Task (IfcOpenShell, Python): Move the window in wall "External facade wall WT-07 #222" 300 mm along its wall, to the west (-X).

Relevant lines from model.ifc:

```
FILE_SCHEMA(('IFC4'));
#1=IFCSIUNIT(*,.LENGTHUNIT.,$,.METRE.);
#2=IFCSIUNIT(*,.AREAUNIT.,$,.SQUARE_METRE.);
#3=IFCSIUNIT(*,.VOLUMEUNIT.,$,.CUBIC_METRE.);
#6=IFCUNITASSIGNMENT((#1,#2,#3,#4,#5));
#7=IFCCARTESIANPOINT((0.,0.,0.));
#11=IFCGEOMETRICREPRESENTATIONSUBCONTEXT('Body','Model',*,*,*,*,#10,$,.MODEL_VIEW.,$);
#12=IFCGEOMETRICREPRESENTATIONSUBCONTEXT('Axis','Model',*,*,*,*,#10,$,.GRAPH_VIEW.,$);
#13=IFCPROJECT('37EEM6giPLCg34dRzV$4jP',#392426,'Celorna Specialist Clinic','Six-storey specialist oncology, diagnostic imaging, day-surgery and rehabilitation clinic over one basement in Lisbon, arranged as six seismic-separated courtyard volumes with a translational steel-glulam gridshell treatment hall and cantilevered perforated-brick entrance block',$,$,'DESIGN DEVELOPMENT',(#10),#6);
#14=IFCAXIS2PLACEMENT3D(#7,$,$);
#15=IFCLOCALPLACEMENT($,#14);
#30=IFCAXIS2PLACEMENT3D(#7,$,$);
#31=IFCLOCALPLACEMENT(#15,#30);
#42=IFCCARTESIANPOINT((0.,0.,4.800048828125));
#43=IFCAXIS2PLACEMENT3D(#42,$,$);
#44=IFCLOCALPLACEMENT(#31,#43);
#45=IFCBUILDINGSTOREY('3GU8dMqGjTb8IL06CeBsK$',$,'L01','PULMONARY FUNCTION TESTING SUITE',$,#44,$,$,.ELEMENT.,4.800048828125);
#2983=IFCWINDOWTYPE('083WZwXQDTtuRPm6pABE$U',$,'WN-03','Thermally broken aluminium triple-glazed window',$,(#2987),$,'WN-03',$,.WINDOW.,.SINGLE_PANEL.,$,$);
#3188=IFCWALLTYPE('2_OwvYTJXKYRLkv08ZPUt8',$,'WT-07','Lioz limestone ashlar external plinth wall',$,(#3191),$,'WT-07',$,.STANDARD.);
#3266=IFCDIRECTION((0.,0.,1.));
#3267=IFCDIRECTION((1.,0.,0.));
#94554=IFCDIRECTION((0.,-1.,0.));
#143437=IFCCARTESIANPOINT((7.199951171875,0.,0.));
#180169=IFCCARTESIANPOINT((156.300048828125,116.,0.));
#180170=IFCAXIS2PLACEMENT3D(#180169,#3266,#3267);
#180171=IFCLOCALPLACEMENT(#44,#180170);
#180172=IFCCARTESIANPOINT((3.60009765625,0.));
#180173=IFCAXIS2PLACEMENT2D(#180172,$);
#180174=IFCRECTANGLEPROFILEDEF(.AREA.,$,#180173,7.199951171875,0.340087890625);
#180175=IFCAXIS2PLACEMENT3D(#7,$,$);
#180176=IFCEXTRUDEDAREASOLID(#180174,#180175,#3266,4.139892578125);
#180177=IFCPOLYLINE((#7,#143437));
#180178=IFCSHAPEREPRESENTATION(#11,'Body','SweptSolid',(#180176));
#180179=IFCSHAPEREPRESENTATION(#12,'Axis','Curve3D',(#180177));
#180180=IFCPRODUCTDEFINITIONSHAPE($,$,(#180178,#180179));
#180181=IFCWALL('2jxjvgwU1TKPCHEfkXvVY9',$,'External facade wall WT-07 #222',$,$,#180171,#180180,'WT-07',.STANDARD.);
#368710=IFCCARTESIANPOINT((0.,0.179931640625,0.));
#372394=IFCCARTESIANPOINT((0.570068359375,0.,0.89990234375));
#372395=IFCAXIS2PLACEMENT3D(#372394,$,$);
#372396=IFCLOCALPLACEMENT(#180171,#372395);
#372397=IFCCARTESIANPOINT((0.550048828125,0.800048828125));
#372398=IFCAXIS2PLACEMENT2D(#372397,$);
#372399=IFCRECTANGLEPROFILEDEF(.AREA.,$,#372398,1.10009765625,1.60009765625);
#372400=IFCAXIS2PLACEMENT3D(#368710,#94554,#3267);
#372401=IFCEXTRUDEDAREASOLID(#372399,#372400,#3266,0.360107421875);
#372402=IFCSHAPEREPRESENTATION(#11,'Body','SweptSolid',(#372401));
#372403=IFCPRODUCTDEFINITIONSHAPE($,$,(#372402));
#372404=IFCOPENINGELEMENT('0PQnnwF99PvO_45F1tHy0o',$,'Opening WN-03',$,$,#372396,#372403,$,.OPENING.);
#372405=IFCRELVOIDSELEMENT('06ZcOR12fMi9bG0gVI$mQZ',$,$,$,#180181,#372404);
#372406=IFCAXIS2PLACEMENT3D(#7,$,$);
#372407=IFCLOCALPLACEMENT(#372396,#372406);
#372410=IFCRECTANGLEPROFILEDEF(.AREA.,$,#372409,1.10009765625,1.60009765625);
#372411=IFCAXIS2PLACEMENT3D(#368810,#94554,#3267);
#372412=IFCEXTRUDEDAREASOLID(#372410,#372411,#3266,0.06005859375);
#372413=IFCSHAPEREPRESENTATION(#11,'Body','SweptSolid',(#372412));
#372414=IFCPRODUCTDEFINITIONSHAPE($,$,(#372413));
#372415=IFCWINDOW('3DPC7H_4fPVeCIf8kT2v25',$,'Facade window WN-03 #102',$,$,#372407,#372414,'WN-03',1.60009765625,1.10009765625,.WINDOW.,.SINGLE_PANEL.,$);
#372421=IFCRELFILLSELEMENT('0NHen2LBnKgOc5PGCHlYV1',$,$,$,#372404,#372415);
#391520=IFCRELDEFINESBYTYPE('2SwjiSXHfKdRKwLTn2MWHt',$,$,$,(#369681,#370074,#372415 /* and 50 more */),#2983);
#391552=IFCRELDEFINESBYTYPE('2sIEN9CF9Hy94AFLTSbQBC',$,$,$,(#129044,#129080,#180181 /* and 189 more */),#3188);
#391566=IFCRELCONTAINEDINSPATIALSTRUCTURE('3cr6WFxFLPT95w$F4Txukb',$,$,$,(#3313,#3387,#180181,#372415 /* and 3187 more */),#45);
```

```python
import ifcopenshell
import ifcopenshell.api.geometry
import ifcopenshell.util.placement

model = ifcopenshell.open("model.ifc")

window = model.by_guid("3DPC7H_4fPVeCIf8kT2v25")
opening = window.FillsVoids[0].RelatingOpeningElement
wall = opening.VoidsElements[0].RelatingBuildingElement

wall_matrix = ifcopenshell.util.placement.get_local_placement(wall.ObjectPlacement)
shift = wall_matrix[:3, 0] * -0.3
before = ifcopenshell.util.placement.get_local_placement(window.ObjectPlacement)[:3, 3].copy()

# The window is placed relative to its opening, so it follows when the opening moves.
matrix = ifcopenshell.util.placement.get_local_placement(opening.ObjectPlacement)
matrix[:3, 3] += shift
ifcopenshell.api.geometry.edit_object_placement(
    model, product=opening, matrix=matrix, is_si=False, should_transform_children=True
)

after = ifcopenshell.util.placement.get_local_placement(window.ObjectPlacement)[:3, 3]
print("window moved by", (after - before).round(3) + 0.0)

model.write("model_v2.ifc")
```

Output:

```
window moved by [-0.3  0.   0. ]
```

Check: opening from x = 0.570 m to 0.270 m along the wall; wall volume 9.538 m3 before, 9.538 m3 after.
